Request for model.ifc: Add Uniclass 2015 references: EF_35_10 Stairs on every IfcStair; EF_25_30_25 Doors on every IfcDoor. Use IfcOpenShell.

First a look at what the model holds.

```python
import ifcopenshell

model = ifcopenshell.open("model.ifc")
print(model.schema)
print("classifications:", [c.Name for c in model.by_type("IfcClassification")])
for ifc_class in ("IfcDoor", "IfcRoof", "IfcStair", "IfcWall", "IfcWindow"):
    print(ifc_class, len(model.by_type(ifc_class)))
```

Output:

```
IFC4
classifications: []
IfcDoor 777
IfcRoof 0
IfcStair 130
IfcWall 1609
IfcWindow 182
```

```python
import ifcopenshell
import ifcopenshell.api.classification

model = ifcopenshell.open("model.ifc")

system = ifcopenshell.api.classification.add_classification(model, classification="Uniclass 2015")

codes = {
    "IfcStair": ("EF_35_10", "Stairs"),
    "IfcDoor": ("EF_25_30_25", "Doors"),
}
for ifc_class, (code, name) in codes.items():
    products = model.by_type(ifc_class)
    ifcopenshell.api.classification.add_reference(
        model, products=products, classification=system, identification=code, name=name
    )
    print(code, len(products))

model.write("model_edited.ifc")
```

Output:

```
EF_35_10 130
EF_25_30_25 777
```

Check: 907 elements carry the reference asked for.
